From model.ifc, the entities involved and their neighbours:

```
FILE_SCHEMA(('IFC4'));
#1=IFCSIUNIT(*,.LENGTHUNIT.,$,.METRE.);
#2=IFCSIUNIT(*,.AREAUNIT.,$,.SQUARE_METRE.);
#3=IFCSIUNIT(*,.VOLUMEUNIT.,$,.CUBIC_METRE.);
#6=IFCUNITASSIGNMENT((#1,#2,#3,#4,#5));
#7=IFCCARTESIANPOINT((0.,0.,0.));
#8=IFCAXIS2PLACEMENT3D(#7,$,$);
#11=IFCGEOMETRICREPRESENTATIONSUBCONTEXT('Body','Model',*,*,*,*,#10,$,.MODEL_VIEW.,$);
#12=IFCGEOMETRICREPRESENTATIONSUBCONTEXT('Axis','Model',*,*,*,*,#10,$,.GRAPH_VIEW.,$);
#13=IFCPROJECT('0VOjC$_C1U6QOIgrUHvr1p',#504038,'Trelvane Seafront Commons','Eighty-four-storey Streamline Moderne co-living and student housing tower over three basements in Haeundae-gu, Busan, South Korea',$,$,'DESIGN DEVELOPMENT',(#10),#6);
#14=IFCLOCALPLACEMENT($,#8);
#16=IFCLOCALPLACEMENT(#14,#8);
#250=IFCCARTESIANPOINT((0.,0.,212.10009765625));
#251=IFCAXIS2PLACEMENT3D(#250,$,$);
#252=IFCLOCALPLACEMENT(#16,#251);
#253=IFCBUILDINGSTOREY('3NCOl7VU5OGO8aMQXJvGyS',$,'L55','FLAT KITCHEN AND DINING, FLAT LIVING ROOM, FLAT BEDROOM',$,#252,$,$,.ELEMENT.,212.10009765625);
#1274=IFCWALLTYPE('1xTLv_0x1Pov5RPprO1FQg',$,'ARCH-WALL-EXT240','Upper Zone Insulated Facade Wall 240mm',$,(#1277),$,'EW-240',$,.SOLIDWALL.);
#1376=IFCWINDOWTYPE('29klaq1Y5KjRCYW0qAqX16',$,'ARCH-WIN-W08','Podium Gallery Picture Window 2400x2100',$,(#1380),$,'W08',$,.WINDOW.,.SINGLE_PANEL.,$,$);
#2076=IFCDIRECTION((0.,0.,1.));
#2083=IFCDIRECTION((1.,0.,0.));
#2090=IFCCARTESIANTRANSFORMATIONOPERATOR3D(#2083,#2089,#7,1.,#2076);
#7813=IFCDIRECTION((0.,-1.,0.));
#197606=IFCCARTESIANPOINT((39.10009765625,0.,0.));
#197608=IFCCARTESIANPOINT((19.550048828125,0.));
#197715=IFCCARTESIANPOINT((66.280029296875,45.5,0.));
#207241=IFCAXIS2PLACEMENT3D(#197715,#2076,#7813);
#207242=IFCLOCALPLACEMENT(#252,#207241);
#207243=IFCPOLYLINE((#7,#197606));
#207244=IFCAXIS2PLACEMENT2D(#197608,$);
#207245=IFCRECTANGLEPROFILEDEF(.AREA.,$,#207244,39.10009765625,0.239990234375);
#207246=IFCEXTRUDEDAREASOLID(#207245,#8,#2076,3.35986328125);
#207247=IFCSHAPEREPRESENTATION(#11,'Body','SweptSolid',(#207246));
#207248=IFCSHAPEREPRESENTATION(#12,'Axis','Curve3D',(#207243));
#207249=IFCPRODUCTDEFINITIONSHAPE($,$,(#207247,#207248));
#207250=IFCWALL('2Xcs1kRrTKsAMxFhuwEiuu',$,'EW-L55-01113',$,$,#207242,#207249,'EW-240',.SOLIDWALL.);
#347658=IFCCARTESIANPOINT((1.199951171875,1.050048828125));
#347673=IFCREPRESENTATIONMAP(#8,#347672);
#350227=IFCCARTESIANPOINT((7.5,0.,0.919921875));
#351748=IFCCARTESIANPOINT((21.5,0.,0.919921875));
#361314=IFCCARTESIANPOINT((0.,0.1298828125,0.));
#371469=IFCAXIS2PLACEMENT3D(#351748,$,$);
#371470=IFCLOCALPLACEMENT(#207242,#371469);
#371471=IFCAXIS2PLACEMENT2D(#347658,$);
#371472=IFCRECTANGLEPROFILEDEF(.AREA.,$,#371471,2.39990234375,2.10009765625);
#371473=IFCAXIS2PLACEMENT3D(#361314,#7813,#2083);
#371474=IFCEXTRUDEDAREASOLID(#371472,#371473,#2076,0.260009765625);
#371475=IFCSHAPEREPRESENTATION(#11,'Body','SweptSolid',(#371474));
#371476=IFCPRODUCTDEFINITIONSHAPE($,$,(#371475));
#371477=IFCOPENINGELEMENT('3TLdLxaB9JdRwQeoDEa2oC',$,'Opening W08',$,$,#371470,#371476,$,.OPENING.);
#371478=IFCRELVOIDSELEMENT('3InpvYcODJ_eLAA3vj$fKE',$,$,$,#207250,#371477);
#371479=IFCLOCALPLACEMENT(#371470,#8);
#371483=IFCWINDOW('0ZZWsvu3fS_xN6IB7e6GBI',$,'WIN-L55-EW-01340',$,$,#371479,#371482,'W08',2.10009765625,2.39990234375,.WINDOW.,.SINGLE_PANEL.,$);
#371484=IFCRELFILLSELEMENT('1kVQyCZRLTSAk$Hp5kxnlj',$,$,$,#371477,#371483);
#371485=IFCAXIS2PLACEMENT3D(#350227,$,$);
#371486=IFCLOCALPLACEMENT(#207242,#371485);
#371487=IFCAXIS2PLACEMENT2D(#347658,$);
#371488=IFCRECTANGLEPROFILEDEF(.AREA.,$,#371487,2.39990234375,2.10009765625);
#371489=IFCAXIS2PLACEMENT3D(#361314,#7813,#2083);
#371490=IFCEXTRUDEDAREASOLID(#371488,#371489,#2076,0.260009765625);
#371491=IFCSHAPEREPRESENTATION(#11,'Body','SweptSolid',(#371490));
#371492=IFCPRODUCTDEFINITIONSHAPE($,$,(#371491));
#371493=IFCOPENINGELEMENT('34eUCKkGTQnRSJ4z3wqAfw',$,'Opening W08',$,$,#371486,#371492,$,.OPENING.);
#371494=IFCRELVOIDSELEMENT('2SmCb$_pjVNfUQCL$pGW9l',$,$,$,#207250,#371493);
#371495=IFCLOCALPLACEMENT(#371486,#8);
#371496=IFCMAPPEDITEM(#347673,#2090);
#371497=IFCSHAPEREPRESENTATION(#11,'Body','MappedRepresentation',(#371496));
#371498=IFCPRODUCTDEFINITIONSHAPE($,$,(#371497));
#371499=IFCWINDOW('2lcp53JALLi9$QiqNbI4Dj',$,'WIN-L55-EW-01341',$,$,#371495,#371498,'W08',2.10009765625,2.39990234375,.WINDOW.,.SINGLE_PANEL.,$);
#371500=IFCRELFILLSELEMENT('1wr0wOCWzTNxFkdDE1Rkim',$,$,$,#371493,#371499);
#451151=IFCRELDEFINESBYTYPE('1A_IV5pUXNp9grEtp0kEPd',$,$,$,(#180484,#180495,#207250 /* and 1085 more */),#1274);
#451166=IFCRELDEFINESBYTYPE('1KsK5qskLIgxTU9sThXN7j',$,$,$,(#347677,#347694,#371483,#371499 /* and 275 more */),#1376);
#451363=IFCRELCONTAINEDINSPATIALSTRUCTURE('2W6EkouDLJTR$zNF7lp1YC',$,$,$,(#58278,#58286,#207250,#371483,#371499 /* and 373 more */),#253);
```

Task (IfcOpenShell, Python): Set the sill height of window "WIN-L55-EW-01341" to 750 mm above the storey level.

```python
import numpy as np
import ifcopenshell
import ifcopenshell.api.geometry
import ifcopenshell.geom
import ifcopenshell.util.element
import ifcopenshell.util.placement
import ifcopenshell.util.shape
import ifcopenshell.util.unit

model = ifcopenshell.open("model.ifc")
unit_scale = ifcopenshell.util.unit.calculate_unit_scale(model)

window = model.by_guid("2lcp53JALLi9$QiqNbI4Dj")
opening = window.FillsVoids[0].RelatingOpeningElement
storey = ifcopenshell.util.element.get_container(window, ifc_class="IfcBuildingStorey")
level = ifcopenshell.util.placement.get_local_placement(storey.ObjectPlacement)[2, 3]

# The opening's origin need not be at the sill, so measure its lowest point.
shape = ifcopenshell.geom.create_shape(ifcopenshell.geom.settings(), opening)
bottom = ifcopenshell.util.shape.get_shape_bottom_elevation(shape, shape.geometry) / unit_scale
dz = level + 0.75 / unit_scale - bottom

shift = np.array([0.0, 0.0, dz])
# The window is placed relative to its opening, so it follows when the opening moves.
matrix = ifcopenshell.util.placement.get_local_placement(opening.ObjectPlacement)
matrix[:3, 3] += shift
ifcopenshell.api.geometry.edit_object_placement(
    model, product=opening, matrix=matrix, is_si=False, should_transform_children=True
)

print(f"moved by {dz * unit_scale:+.3f} m")

model.write("model_edited.ifc")
```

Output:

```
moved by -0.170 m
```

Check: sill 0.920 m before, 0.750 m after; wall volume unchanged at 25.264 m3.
